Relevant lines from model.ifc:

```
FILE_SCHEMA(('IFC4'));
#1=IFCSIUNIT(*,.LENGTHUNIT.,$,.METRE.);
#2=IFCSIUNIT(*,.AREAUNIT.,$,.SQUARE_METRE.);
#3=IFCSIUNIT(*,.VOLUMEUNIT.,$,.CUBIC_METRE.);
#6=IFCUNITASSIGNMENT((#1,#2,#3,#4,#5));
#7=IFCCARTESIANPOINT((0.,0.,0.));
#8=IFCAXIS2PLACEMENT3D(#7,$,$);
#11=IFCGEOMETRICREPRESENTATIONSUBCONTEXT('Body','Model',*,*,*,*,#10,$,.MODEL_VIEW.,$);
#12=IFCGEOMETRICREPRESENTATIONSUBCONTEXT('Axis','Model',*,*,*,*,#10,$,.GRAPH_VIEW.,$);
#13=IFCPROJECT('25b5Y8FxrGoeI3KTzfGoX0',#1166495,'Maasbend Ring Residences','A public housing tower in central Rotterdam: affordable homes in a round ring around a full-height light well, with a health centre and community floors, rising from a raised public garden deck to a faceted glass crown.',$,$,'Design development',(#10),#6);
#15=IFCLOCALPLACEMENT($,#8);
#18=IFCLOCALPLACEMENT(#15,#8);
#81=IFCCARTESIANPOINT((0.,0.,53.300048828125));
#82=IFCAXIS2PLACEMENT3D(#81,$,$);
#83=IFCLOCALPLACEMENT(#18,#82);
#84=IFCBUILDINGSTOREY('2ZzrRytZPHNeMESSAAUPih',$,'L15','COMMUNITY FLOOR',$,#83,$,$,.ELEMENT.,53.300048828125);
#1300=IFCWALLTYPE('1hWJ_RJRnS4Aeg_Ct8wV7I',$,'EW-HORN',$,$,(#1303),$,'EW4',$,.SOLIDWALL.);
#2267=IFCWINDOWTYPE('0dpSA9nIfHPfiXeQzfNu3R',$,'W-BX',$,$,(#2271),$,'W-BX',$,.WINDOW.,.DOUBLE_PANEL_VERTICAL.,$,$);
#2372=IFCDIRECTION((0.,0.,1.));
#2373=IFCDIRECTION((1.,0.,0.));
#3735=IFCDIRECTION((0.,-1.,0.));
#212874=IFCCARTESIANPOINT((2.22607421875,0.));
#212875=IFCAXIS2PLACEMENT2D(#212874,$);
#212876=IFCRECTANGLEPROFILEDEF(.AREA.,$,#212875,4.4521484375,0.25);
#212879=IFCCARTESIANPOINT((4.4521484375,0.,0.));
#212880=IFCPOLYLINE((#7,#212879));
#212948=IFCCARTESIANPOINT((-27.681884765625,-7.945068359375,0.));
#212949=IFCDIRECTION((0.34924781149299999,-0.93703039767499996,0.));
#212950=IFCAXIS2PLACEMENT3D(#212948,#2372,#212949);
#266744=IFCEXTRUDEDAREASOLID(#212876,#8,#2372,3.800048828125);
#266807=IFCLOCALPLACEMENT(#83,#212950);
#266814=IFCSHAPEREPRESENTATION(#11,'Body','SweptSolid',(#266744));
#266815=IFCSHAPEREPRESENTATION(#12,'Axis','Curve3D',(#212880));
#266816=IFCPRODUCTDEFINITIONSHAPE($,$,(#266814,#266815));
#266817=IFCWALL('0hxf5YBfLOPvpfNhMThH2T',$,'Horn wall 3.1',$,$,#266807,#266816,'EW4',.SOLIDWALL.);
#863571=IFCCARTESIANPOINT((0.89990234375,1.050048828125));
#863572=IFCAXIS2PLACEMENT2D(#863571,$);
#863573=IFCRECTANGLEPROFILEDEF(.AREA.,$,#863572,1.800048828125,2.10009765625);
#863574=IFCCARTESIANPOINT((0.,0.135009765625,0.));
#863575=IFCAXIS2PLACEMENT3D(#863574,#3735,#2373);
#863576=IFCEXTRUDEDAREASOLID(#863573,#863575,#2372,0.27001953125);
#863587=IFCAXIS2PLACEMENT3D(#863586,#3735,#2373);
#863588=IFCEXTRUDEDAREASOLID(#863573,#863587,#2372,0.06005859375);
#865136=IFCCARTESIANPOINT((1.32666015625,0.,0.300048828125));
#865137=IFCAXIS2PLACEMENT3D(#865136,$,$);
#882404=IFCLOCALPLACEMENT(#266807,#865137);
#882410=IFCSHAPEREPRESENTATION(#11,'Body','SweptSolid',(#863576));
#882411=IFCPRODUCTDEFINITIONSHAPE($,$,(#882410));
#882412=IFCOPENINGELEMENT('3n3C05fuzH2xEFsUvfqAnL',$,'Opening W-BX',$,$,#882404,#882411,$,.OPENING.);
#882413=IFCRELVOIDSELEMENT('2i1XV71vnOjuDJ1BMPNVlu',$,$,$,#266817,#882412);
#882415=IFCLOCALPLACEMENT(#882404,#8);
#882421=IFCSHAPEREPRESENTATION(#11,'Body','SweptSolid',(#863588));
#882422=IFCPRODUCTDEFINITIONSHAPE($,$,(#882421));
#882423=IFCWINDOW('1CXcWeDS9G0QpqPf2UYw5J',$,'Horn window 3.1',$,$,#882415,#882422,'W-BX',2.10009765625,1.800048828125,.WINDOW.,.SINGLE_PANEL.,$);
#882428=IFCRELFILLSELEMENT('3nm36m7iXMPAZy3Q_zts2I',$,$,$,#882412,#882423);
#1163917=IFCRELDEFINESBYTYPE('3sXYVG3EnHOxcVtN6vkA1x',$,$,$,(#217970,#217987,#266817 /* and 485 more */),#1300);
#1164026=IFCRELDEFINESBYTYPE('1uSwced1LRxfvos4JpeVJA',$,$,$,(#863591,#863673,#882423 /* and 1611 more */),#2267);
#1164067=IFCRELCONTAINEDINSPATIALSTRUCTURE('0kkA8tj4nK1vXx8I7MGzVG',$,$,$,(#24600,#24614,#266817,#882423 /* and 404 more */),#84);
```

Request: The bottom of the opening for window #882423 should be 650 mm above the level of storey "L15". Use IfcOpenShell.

```python
import numpy as np
import ifcopenshell
import ifcopenshell.api.geometry
import ifcopenshell.geom
import ifcopenshell.util.element
import ifcopenshell.util.placement
import ifcopenshell.util.shape
import ifcopenshell.util.unit

model = ifcopenshell.open("model.ifc")
unit_scale = ifcopenshell.util.unit.calculate_unit_scale(model)

window = model.by_guid("1CXcWeDS9G0QpqPf2UYw5J")
opening = window.FillsVoids[0].RelatingOpeningElement
storey = ifcopenshell.util.element.get_container(window, ifc_class="IfcBuildingStorey")
level = ifcopenshell.util.placement.get_local_placement(storey.ObjectPlacement)[2, 3]

# The opening's origin need not be at the sill, so measure its lowest point.
shape = ifcopenshell.geom.create_shape(ifcopenshell.geom.settings(), opening)
bottom = ifcopenshell.util.shape.get_shape_bottom_elevation(shape, shape.geometry) / unit_scale
dz = level + 0.65 - bottom

shift = np.array([0.0, 0.0, dz])
# The window is placed relative to its opening, so it follows when the opening moves.
matrix = ifcopenshell.util.placement.get_local_placement(opening.ObjectPlacement)
matrix[:3, 3] += shift
ifcopenshell.api.geometry.edit_object_placement(
    model, product=opening, matrix=matrix, is_si=False, should_transform_children=True
)

print(f"moved by {dz * unit_scale:+.3f} m")

model.write("model-out.ifc")
```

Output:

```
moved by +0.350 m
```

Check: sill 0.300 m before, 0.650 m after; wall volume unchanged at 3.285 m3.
